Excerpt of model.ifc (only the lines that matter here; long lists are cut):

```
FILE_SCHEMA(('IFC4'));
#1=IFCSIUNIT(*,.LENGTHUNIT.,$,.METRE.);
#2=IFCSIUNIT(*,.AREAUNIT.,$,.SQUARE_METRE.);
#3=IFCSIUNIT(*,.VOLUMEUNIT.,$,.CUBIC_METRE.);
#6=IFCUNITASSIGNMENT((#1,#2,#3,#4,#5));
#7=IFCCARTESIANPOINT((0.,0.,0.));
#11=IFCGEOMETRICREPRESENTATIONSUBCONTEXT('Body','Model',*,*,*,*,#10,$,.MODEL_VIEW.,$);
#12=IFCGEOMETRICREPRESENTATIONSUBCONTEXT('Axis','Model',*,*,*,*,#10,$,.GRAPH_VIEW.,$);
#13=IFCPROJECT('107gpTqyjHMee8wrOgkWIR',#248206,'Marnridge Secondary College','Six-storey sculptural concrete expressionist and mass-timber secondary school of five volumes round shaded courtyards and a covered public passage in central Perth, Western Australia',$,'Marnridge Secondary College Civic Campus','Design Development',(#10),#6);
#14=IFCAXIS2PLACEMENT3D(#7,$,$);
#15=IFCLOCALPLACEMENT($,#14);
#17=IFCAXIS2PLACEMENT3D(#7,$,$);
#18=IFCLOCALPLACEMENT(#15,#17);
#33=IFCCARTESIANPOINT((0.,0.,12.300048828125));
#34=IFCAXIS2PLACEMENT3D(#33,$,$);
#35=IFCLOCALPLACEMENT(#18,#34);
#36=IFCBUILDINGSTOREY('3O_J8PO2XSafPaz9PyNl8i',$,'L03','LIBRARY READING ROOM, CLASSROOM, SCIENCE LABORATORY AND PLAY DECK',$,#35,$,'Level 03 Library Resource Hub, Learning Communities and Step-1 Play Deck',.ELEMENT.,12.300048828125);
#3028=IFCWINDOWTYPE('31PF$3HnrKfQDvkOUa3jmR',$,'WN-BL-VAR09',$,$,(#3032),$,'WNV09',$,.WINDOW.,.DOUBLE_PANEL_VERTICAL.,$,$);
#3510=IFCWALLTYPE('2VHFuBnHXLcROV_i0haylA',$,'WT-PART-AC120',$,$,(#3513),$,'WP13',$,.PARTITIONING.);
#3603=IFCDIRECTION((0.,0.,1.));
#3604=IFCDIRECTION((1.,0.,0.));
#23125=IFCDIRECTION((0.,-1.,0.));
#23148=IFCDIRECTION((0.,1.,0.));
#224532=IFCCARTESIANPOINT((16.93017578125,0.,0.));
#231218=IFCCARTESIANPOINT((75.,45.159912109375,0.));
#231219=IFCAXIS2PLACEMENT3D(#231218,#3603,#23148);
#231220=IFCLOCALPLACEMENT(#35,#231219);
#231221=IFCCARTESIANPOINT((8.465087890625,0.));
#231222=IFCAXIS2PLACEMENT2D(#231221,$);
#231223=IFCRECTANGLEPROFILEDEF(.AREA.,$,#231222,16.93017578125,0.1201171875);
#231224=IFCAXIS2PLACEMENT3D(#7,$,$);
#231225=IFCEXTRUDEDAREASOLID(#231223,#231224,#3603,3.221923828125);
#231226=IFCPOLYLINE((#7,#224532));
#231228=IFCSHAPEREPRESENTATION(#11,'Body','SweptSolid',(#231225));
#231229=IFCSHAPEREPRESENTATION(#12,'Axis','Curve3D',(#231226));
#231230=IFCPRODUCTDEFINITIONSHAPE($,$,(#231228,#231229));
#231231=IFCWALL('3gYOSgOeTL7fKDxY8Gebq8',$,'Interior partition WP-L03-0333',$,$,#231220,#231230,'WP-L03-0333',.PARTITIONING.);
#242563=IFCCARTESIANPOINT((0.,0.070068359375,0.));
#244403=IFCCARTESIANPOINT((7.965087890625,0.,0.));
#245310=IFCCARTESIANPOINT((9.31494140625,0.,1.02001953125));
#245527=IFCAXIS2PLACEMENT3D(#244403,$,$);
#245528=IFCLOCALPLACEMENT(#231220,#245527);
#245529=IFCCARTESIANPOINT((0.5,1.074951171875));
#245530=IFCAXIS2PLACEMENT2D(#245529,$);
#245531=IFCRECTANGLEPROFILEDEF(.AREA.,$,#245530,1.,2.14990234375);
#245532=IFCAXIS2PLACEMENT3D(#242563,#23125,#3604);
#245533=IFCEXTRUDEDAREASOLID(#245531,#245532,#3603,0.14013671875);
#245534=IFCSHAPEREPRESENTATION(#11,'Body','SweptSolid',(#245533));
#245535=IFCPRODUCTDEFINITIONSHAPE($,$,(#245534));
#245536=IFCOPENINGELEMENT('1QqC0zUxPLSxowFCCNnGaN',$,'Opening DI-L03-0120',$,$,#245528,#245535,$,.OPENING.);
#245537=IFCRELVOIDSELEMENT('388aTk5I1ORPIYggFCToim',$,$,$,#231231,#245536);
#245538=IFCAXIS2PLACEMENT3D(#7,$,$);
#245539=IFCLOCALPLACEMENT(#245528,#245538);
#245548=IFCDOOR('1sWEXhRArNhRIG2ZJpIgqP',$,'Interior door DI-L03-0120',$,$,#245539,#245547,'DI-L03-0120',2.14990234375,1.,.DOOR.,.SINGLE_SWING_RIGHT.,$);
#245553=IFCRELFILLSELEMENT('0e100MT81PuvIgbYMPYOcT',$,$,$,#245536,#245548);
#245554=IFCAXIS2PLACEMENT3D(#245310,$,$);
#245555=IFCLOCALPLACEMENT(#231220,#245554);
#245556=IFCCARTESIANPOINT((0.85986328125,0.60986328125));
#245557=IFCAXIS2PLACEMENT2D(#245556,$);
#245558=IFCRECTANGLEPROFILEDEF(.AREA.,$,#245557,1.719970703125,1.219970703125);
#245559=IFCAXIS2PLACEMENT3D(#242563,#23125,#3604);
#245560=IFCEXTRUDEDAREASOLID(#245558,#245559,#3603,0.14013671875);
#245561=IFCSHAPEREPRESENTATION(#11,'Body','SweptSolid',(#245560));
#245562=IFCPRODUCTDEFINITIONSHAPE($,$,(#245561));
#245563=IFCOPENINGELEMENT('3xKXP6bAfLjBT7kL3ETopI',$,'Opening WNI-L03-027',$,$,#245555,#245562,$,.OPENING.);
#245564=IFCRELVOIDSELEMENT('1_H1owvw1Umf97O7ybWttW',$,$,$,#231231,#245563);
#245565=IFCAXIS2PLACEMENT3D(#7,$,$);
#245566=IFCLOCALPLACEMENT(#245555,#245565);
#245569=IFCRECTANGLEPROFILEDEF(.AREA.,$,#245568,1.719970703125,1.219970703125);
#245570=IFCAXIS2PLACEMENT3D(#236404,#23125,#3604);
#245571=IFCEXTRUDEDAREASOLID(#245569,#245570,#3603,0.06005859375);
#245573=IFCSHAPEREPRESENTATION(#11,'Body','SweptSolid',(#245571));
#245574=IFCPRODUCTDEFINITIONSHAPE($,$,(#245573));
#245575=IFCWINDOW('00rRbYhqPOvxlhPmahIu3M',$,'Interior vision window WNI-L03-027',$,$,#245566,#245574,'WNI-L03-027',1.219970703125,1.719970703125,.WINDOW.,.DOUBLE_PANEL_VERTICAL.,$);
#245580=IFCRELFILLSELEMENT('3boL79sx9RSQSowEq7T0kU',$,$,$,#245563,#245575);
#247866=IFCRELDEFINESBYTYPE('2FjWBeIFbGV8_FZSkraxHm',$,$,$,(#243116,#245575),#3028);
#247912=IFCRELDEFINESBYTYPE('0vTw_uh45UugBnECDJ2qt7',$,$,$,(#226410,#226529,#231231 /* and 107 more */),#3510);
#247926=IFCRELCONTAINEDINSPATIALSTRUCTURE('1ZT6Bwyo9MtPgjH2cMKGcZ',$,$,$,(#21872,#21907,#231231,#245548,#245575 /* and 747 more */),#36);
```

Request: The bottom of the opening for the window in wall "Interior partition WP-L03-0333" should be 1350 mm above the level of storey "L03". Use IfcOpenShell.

```python
import numpy as np
import ifcopenshell
import ifcopenshell.api.geometry
import ifcopenshell.geom
import ifcopenshell.util.element
import ifcopenshell.util.placement
import ifcopenshell.util.shape
import ifcopenshell.util.unit

model = ifcopenshell.open("model.ifc")
unit_scale = ifcopenshell.util.unit.calculate_unit_scale(model)

window = model.by_guid("00rRbYhqPOvxlhPmahIu3M")
opening = window.FillsVoids[0].RelatingOpeningElement
storey = ifcopenshell.util.element.get_container(window, ifc_class="IfcBuildingStorey")
level = ifcopenshell.util.placement.get_local_placement(storey.ObjectPlacement)[2, 3]

# The opening's origin need not be at the sill, so measure its lowest point.
shape = ifcopenshell.geom.create_shape(ifcopenshell.geom.settings(), opening)
bottom = ifcopenshell.util.shape.get_shape_bottom_elevation(shape, shape.geometry) / unit_scale
dz = level + 1.35 / unit_scale - bottom

shift = np.array([0.0, 0.0, dz])
# The window is placed relative to its opening, so it follows when the opening moves.
matrix = ifcopenshell.util.placement.get_local_placement(opening.ObjectPlacement)
matrix[:3, 3] += shift
ifcopenshell.api.geometry.edit_object_placement(
    model, product=opening, matrix=matrix, is_si=False, should_transform_children=True
)

print(f"moved by {dz * unit_scale:+.3f} m")

model.write("model-out.ifc")
```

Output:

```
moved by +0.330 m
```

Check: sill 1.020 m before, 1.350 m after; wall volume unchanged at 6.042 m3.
